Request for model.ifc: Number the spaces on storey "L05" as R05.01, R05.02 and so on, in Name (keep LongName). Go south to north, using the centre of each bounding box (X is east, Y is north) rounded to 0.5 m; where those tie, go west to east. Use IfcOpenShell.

First a look at what the model holds.

```python
import ifcopenshell
import ifcopenshell.util.element
import ifcopenshell.util.placement

model = ifcopenshell.open("model.ifc")
print(model.schema)
storey = next(s for s in model.by_type("IfcBuildingStorey") if s.Name == "L05")
spaces = [e for e in ifcopenshell.util.element.get_decomposition(storey) if e.is_a("IfcSpace")]
for e in sorted(spaces, key=lambda e: e.id()):
    origin = ifcopenshell.util.placement.get_local_placement(e.ObjectPlacement)[:3, 3]
    print(e.id(), e.Name, e.LongName, origin.round(2) + 0.0, sep=" | ")
```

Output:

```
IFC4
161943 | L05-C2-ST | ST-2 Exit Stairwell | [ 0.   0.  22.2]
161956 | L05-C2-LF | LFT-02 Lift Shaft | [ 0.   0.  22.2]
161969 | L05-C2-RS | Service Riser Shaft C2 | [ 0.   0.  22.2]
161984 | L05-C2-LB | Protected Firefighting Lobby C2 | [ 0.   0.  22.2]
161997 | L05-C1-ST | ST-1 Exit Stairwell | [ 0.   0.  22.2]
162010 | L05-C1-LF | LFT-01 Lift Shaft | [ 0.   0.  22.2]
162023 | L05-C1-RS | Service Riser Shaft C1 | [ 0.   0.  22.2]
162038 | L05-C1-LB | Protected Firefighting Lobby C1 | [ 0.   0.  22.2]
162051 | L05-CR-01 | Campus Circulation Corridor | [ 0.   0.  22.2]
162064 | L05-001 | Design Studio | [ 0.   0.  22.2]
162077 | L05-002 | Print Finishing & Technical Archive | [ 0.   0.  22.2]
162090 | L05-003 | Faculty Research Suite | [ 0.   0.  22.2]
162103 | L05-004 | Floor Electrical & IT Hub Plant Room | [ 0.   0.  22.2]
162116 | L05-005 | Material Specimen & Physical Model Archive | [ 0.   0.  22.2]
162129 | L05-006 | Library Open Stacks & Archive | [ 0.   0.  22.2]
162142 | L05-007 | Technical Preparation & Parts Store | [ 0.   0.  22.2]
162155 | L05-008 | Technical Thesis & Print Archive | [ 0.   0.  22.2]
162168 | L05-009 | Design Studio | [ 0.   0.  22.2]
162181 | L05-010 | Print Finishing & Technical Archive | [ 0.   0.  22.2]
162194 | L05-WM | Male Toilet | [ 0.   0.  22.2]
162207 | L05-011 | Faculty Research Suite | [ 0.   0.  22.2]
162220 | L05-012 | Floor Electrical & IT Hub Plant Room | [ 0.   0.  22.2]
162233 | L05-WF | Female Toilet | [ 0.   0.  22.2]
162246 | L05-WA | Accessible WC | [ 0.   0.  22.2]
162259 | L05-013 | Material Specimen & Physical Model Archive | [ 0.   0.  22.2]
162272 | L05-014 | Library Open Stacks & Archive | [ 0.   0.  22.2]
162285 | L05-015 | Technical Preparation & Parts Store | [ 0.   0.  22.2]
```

```python
import ifcopenshell
import ifcopenshell.geom
import ifcopenshell.util.element
import ifcopenshell.util.shape

model = ifcopenshell.open("model.ifc")
settings = ifcopenshell.geom.settings()
settings.set("use-world-coords", True)


def centre(element):
    shape = ifcopenshell.geom.create_shape(settings, element)
    return ifcopenshell.util.shape.get_bbox_centroid(shape.geometry)


storey = next(s for s in model.by_type("IfcBuildingStorey") if s.Name == "L05")
spaces = [e for e in ifcopenshell.util.element.get_decomposition(storey) if e.is_a("IfcSpace")]

# Insertion points can sit at a corner or the storey origin, so sort by the geometry (in metres).
centres = {e: centre(e) for e in spaces}
spaces.sort(key=lambda e: (round(centres[e][1] / 0.5), centres[e][0]))

for i, e in enumerate(spaces, start=1):
    number = f"R05.{i:02d}"
    e.Name = number
    print(e.id(), number)

model.write("model_rev.ifc")
```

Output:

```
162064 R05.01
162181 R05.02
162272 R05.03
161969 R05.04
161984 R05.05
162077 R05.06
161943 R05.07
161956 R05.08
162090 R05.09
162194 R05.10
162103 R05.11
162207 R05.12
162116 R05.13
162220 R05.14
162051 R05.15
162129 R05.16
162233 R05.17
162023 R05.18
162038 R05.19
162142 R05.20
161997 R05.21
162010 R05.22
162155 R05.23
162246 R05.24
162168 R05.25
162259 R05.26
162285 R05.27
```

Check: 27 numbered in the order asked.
